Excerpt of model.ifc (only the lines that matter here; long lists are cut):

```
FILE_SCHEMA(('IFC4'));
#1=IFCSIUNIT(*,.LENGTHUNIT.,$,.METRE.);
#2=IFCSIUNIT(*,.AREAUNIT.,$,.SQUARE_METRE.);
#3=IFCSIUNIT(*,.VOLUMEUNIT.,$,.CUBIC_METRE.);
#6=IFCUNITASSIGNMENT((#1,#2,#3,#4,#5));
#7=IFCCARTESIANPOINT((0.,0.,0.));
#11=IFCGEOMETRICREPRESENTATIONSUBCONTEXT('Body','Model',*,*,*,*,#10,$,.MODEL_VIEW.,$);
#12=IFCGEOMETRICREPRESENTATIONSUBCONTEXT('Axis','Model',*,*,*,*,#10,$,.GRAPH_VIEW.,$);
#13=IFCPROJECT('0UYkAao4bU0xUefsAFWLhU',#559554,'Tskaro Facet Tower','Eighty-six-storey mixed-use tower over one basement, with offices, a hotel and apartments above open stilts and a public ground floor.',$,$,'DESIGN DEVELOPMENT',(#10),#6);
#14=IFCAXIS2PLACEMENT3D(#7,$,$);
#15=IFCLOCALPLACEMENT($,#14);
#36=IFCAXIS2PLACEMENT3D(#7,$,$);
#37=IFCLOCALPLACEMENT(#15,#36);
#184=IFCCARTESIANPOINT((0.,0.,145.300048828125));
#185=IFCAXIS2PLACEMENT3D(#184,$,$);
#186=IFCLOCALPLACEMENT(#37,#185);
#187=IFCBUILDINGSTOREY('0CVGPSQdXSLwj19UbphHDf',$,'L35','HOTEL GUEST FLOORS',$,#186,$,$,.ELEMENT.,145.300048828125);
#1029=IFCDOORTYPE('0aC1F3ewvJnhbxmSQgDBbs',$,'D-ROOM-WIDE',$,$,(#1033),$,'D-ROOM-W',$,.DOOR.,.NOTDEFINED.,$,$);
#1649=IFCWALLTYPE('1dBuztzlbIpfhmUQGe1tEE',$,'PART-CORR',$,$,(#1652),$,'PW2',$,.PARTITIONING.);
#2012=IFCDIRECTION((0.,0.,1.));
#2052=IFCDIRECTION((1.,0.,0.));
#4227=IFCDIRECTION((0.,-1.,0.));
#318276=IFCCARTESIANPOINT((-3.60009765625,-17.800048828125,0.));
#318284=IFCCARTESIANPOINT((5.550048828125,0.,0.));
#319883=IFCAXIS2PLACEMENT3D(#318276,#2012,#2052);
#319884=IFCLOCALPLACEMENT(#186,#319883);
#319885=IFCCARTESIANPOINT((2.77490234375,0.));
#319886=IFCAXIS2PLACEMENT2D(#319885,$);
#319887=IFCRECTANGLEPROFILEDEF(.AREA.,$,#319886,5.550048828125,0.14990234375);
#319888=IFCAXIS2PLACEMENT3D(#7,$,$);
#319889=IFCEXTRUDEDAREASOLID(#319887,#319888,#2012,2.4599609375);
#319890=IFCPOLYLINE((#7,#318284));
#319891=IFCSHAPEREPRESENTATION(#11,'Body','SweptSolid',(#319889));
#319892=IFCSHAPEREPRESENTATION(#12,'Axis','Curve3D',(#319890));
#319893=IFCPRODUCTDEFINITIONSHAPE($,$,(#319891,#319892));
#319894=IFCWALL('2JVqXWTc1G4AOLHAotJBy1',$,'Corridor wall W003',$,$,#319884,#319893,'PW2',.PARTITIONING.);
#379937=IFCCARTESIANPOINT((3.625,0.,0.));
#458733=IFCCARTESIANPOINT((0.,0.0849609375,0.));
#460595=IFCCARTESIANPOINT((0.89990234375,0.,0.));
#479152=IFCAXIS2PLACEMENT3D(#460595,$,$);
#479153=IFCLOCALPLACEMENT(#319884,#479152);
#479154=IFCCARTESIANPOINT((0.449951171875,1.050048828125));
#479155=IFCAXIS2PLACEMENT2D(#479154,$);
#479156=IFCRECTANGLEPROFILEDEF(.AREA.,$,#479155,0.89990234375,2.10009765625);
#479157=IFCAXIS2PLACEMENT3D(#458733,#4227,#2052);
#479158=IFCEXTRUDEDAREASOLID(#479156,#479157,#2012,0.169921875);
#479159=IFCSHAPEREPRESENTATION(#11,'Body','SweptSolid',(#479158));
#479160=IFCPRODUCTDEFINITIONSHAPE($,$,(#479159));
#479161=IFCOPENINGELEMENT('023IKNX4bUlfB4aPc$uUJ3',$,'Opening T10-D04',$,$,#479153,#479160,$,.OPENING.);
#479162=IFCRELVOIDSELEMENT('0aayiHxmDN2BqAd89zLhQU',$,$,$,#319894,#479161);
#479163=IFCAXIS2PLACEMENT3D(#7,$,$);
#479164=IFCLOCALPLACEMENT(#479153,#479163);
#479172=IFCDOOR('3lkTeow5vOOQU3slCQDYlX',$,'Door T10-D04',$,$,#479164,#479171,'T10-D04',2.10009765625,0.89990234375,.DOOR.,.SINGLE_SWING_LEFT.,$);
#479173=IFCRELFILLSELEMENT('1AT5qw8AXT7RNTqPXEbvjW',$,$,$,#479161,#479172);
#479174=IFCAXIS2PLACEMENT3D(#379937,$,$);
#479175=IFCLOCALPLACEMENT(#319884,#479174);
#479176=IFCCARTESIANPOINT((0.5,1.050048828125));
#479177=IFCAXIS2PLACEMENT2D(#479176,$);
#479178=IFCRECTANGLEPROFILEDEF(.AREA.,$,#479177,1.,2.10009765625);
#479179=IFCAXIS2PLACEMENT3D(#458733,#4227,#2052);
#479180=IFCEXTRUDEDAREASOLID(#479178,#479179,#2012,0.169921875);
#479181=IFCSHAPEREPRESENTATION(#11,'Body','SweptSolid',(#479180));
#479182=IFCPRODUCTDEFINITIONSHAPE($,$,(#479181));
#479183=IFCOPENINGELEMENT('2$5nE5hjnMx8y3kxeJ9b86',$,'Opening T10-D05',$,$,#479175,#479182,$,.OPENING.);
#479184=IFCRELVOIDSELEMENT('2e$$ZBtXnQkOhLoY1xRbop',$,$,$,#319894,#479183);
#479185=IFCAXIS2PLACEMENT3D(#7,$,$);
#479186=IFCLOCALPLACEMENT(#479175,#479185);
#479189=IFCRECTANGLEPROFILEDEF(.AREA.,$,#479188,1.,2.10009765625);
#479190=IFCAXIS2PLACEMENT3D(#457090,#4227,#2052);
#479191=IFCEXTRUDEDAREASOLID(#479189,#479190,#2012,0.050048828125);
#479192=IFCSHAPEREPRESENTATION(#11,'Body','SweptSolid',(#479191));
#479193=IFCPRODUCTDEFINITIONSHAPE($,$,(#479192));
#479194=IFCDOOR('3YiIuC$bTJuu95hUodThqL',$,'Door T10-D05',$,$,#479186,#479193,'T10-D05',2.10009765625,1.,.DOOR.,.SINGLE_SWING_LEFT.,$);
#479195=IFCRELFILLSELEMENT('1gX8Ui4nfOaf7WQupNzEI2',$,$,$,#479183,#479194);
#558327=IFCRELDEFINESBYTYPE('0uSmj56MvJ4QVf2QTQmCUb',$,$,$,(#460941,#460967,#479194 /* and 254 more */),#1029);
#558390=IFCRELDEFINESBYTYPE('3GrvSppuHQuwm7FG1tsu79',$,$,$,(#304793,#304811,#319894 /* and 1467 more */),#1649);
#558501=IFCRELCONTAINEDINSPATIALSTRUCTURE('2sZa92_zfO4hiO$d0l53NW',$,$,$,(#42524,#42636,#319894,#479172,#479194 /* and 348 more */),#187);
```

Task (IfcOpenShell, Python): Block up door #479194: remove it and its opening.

```python
import ifcopenshell
import ifcopenshell.api.feature
import ifcopenshell.api.root
import ifcopenshell.geom
import ifcopenshell.util.shape

model = ifcopenshell.open("model.ifc")
settings = ifcopenshell.geom.settings()


def volume(element):
    """Net volume in cubic metres, openings subtracted."""
    shape = ifcopenshell.geom.create_shape(settings, element)
    return ifcopenshell.util.shape.get_volume(shape.geometry)


door = model.by_guid("3YiIuC$bTJuu95hUodThqL")
opening = door.FillsVoids[0].RelatingOpeningElement
wall = opening.VoidsElements[0].RelatingBuildingElement
before = volume(wall)

ifcopenshell.api.root.remove_product(model, product=door)
ifcopenshell.api.feature.remove_feature(model, feature=opening)

after = volume(wall)

print(f"wall volume {before:.3f} -> {after:.3f} m3")

model.write("model_edited.ifc")
```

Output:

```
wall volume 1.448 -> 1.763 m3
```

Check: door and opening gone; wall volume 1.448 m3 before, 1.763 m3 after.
